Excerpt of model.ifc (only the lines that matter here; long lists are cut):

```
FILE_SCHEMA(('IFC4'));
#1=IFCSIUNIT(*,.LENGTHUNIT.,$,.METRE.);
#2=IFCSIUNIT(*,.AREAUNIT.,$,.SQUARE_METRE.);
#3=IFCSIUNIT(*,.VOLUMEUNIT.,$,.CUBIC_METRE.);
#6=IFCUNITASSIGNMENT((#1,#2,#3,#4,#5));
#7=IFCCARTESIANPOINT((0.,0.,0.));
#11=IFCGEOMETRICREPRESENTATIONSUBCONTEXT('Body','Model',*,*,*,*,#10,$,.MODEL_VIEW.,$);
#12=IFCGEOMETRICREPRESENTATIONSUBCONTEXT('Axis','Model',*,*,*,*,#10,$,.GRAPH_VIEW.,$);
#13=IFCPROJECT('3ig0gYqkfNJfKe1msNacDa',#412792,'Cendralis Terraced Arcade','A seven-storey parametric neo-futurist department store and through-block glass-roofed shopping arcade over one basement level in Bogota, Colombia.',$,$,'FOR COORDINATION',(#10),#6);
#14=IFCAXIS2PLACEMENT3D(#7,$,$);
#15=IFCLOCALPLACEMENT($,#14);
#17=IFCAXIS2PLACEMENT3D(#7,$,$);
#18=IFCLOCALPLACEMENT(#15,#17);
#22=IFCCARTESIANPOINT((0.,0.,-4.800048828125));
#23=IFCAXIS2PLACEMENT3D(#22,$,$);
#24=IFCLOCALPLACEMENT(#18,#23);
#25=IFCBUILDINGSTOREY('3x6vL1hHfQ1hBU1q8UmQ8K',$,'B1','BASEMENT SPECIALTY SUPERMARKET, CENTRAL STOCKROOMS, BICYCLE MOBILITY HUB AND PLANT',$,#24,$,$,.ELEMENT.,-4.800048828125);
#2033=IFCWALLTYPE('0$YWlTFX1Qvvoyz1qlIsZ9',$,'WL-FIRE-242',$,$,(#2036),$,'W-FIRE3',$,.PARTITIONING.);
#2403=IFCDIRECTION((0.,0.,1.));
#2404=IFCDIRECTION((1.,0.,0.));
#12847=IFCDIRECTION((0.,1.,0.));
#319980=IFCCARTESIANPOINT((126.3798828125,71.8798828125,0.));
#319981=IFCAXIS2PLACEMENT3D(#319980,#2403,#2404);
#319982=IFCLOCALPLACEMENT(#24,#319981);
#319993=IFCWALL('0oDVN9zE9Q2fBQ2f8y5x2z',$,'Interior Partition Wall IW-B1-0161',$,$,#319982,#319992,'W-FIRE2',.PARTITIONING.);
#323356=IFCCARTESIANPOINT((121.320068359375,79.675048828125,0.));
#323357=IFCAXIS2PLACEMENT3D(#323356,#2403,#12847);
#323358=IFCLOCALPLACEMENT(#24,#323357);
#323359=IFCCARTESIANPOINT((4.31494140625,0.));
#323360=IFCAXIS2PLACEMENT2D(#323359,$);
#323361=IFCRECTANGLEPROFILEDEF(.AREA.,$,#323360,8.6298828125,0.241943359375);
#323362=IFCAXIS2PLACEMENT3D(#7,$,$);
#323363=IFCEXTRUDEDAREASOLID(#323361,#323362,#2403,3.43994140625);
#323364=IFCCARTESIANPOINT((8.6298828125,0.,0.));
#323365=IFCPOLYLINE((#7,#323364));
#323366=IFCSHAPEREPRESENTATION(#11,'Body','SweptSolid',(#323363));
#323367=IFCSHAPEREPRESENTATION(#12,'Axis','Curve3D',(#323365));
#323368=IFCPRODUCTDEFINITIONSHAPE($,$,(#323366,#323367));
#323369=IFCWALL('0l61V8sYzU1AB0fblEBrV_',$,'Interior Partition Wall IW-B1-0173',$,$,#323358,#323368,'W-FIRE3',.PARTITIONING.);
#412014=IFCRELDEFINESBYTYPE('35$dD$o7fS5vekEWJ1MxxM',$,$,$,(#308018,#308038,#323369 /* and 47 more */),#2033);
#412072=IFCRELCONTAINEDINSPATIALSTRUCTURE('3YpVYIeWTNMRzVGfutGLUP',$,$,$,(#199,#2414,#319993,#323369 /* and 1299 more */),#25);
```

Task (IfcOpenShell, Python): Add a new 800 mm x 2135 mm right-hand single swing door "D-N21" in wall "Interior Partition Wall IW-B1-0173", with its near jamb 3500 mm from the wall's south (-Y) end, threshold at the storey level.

```python
import numpy as np
import ifcopenshell
import ifcopenshell.api.feature
import ifcopenshell.api.geometry
import ifcopenshell.api.root
import ifcopenshell.api.spatial
import ifcopenshell.geom
import ifcopenshell.util.element
import ifcopenshell.util.placement
import ifcopenshell.util.representation
import ifcopenshell.util.shape
import ifcopenshell.util.unit

model = ifcopenshell.open("model.ifc")
unit_scale = ifcopenshell.util.unit.calculate_unit_scale(model)
settings = ifcopenshell.geom.settings()


def volume(element):
    """Net volume in cubic metres, openings subtracted."""
    shape = ifcopenshell.geom.create_shape(settings, element)
    return ifcopenshell.util.shape.get_volume(shape.geometry)


wall = model.by_guid("0l61V8sYzU1AB0fblEBrV_")
storey = ifcopenshell.util.element.get_container(wall, ifc_class="IfcBuildingStorey")
context = ifcopenshell.util.representation.get_context(model, "Model", "Body", "MODEL_VIEW")
before = volume(wall)

width, height, from_end, sill = 0.8, 2.135, 3.5, 0.0  # metres

# The wall runs along its own X axis, and the end named is its -X end.
wall_shape = ifcopenshell.geom.create_shape(settings, wall)
x, y, z = ifcopenshell.util.shape.get_vertices(wall_shape.geometry).T
start = x.min() + from_end
face, thickness = float(y.min()), float(y.max() - y.min())
wall_matrix = ifcopenshell.util.placement.get_local_placement(wall.ObjectPlacement)
level = ifcopenshell.util.placement.get_local_placement(storey.ObjectPlacement)[2, 3]


def in_wall(x, y):
    """Placement at x, y metres in the wall's axes, at sill height."""
    matrix = wall_matrix.copy()
    matrix[:, 3] = wall_matrix @ np.array([x / unit_scale, y / unit_scale, 0.0, 1.0])
    matrix[2, 3] = level + sill / unit_scale
    return matrix


# Opening: a box that overshoots both wall faces by 50 mm.
opening = ifcopenshell.api.root.create_entity(model, ifc_class="IfcOpeningElement", predefined_type="OPENING")
box = ifcopenshell.api.geometry.add_wall_representation(
    model, context=context, length=width, height=height, thickness=thickness + 0.1
)
ifcopenshell.api.geometry.assign_representation(model, product=opening, representation=box)
ifcopenshell.api.geometry.edit_object_placement(model, product=opening, matrix=in_wall(start, face - 0.05), is_si=False)
ifcopenshell.api.feature.add_feature(model, feature=opening, element=wall)

door = ifcopenshell.api.root.create_entity(model, ifc_class="IfcDoor", name="D-N21", predefined_type="DOOR")
door.OverallWidth, door.OverallHeight = width / unit_scale, height / unit_scale
door.OperationType = "SINGLE_SWING_RIGHT"
body = ifcopenshell.api.geometry.add_door_representation(
    model,
    context=context,
    overall_width=door.OverallWidth,
    overall_height=door.OverallHeight,
    operation_type="SINGLE_SWING_RIGHT",
    lining_properties={"LiningDepth": thickness / unit_scale, "ThresholdDepth": thickness / unit_scale},
)
ifcopenshell.api.geometry.assign_representation(model, product=door, representation=body)
ifcopenshell.api.spatial.assign_container(model, products=[door], relating_structure=storey)
ifcopenshell.api.feature.add_filling(model, opening=opening, element=door)

# The lining spans the wall, so the door starts at the wall face.
ifcopenshell.api.geometry.edit_object_placement(model, product=door, matrix=in_wall(start, face), is_si=False)

after = volume(wall)

print(f"wall volume {before:.3f} -> {after:.3f} m3")

model.write("model-out.ifc")
```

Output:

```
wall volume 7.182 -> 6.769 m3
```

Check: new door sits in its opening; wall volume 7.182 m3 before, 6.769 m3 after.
